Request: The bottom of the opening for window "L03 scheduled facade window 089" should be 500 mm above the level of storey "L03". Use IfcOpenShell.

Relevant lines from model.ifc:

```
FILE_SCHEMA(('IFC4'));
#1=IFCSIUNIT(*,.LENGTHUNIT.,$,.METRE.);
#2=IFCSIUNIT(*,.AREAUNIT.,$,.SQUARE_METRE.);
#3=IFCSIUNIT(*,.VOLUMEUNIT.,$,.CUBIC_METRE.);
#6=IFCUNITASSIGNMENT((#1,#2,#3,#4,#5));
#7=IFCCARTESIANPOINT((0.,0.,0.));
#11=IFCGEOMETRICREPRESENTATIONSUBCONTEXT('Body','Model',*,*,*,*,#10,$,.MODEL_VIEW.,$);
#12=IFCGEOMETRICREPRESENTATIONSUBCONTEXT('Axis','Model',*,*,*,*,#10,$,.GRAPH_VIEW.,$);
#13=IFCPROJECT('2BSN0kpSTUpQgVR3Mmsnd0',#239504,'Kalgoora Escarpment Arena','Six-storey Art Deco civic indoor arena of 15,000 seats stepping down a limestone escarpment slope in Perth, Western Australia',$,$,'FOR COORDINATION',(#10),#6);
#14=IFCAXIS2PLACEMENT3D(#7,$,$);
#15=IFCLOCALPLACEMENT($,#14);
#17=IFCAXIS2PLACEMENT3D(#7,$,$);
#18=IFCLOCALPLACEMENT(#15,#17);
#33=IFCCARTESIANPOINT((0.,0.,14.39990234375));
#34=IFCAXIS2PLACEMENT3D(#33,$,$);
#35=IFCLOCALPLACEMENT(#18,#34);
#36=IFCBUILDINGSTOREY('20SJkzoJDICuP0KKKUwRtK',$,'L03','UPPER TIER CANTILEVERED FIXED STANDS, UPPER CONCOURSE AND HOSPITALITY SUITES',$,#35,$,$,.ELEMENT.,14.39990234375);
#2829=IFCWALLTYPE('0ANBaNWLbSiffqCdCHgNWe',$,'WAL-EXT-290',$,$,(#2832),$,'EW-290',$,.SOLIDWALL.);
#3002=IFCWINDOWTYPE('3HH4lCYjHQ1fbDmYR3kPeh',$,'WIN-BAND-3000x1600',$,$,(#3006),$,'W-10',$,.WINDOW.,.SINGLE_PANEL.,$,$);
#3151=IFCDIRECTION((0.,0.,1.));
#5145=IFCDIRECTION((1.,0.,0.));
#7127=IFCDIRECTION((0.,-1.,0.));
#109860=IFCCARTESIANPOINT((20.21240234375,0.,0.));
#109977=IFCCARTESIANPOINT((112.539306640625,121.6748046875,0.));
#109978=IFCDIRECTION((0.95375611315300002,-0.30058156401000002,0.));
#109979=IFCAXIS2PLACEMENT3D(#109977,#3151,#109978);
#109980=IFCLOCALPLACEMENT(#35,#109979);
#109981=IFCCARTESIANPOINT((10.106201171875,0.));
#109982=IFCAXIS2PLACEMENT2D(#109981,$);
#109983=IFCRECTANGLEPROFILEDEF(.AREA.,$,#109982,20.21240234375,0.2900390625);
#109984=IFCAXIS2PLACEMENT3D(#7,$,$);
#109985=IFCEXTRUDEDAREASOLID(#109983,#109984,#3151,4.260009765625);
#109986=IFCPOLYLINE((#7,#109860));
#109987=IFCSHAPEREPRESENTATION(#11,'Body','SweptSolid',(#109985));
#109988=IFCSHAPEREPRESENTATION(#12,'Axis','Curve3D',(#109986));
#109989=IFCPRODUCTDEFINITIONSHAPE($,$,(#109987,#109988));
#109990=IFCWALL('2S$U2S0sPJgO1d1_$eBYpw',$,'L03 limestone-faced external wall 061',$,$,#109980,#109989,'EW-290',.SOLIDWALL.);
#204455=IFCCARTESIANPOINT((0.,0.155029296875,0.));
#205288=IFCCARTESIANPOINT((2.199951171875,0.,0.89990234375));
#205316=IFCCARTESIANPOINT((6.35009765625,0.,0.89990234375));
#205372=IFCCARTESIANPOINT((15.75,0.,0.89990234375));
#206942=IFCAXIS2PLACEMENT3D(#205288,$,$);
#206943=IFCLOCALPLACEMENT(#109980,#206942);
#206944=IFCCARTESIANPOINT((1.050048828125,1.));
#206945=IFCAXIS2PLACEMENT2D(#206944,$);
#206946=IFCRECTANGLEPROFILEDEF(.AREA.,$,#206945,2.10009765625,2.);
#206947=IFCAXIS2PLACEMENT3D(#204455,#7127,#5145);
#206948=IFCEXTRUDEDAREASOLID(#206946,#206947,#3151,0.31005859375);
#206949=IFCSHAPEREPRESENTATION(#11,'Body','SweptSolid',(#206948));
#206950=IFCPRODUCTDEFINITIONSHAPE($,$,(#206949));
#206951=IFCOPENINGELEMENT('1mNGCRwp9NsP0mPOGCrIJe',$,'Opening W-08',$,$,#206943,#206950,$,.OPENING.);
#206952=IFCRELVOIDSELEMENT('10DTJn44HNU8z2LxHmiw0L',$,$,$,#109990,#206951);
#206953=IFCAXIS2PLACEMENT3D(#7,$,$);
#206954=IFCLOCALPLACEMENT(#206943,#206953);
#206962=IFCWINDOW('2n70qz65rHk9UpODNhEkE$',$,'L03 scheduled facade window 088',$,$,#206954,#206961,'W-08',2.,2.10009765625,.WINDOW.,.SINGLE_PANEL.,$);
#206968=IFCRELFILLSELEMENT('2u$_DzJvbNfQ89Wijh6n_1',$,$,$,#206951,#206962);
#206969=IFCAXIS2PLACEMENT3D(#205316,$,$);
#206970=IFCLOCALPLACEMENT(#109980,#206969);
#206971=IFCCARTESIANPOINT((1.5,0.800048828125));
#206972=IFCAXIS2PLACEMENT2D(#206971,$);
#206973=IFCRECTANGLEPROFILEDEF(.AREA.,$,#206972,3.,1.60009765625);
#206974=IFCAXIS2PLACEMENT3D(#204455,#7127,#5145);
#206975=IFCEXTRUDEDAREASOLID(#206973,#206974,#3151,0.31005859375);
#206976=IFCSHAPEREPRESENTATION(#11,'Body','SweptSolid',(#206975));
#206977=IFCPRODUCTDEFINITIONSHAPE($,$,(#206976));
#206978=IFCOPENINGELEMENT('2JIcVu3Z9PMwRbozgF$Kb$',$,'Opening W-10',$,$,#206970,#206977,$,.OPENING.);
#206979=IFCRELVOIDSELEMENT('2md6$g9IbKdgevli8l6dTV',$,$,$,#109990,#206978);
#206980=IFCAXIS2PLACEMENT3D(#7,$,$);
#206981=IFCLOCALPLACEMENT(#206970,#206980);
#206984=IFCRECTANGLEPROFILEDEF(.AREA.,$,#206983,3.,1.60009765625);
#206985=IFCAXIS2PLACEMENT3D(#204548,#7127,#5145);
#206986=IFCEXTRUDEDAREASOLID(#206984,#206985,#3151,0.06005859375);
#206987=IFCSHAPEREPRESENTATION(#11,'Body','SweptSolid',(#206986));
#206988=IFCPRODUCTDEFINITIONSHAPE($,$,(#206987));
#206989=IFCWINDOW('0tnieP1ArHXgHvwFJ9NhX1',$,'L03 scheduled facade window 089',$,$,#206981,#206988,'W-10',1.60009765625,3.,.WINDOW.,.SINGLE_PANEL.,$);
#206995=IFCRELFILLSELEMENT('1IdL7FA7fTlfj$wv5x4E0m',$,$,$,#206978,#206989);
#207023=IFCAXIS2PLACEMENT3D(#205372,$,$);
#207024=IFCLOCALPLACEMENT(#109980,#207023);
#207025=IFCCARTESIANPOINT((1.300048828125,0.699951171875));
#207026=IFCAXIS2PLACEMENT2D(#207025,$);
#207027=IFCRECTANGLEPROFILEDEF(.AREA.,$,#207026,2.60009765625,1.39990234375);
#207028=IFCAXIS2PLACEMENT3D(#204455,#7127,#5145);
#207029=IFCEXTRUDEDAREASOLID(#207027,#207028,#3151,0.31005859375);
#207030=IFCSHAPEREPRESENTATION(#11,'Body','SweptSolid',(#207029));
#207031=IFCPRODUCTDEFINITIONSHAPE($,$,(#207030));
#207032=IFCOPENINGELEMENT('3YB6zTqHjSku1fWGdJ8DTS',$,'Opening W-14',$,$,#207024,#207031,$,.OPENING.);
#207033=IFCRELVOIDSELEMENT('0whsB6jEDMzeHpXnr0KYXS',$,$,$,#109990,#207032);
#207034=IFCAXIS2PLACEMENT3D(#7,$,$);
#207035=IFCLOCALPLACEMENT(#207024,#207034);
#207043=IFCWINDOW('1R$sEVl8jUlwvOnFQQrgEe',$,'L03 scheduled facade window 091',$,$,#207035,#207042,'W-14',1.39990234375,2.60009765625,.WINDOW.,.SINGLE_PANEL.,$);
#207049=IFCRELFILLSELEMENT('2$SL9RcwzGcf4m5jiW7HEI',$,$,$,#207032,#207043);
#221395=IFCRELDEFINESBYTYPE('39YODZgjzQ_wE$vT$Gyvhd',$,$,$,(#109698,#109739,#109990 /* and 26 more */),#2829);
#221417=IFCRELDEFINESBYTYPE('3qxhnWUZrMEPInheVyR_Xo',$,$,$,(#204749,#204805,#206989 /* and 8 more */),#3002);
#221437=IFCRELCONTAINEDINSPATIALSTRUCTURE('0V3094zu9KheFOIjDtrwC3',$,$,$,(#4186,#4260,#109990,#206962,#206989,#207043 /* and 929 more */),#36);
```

```python
import numpy as np
import ifcopenshell
import ifcopenshell.api.geometry
import ifcopenshell.geom
import ifcopenshell.util.element
import ifcopenshell.util.placement
import ifcopenshell.util.shape
import ifcopenshell.util.unit

model = ifcopenshell.open("model.ifc")
unit_scale = ifcopenshell.util.unit.calculate_unit_scale(model)

window = model.by_id(206989)
opening = window.FillsVoids[0].RelatingOpeningElement
storey = ifcopenshell.util.element.get_container(window, ifc_class="IfcBuildingStorey")
level = ifcopenshell.util.placement.get_local_placement(storey.ObjectPlacement)[2, 3]

# The opening's origin need not be at the sill, so measure its lowest point.
shape = ifcopenshell.geom.create_shape(ifcopenshell.geom.settings(), opening)
bottom = ifcopenshell.util.shape.get_shape_bottom_elevation(shape, shape.geometry) / unit_scale
dz = level + 0.5 / unit_scale - bottom

shift = np.array([0.0, 0.0, dz])
# The window is placed relative to its opening, so it follows when the opening moves.
matrix = ifcopenshell.util.placement.get_local_placement(opening.ObjectPlacement)
matrix[:3, 3] += shift
ifcopenshell.api.geometry.edit_object_placement(
    model, product=opening, matrix=matrix, is_si=False, should_transform_children=True
)

print(f"moved by {dz * unit_scale:+.3f} m")

model.write("model_edited.ifc")
```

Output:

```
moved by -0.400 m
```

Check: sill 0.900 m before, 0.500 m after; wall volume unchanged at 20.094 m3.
